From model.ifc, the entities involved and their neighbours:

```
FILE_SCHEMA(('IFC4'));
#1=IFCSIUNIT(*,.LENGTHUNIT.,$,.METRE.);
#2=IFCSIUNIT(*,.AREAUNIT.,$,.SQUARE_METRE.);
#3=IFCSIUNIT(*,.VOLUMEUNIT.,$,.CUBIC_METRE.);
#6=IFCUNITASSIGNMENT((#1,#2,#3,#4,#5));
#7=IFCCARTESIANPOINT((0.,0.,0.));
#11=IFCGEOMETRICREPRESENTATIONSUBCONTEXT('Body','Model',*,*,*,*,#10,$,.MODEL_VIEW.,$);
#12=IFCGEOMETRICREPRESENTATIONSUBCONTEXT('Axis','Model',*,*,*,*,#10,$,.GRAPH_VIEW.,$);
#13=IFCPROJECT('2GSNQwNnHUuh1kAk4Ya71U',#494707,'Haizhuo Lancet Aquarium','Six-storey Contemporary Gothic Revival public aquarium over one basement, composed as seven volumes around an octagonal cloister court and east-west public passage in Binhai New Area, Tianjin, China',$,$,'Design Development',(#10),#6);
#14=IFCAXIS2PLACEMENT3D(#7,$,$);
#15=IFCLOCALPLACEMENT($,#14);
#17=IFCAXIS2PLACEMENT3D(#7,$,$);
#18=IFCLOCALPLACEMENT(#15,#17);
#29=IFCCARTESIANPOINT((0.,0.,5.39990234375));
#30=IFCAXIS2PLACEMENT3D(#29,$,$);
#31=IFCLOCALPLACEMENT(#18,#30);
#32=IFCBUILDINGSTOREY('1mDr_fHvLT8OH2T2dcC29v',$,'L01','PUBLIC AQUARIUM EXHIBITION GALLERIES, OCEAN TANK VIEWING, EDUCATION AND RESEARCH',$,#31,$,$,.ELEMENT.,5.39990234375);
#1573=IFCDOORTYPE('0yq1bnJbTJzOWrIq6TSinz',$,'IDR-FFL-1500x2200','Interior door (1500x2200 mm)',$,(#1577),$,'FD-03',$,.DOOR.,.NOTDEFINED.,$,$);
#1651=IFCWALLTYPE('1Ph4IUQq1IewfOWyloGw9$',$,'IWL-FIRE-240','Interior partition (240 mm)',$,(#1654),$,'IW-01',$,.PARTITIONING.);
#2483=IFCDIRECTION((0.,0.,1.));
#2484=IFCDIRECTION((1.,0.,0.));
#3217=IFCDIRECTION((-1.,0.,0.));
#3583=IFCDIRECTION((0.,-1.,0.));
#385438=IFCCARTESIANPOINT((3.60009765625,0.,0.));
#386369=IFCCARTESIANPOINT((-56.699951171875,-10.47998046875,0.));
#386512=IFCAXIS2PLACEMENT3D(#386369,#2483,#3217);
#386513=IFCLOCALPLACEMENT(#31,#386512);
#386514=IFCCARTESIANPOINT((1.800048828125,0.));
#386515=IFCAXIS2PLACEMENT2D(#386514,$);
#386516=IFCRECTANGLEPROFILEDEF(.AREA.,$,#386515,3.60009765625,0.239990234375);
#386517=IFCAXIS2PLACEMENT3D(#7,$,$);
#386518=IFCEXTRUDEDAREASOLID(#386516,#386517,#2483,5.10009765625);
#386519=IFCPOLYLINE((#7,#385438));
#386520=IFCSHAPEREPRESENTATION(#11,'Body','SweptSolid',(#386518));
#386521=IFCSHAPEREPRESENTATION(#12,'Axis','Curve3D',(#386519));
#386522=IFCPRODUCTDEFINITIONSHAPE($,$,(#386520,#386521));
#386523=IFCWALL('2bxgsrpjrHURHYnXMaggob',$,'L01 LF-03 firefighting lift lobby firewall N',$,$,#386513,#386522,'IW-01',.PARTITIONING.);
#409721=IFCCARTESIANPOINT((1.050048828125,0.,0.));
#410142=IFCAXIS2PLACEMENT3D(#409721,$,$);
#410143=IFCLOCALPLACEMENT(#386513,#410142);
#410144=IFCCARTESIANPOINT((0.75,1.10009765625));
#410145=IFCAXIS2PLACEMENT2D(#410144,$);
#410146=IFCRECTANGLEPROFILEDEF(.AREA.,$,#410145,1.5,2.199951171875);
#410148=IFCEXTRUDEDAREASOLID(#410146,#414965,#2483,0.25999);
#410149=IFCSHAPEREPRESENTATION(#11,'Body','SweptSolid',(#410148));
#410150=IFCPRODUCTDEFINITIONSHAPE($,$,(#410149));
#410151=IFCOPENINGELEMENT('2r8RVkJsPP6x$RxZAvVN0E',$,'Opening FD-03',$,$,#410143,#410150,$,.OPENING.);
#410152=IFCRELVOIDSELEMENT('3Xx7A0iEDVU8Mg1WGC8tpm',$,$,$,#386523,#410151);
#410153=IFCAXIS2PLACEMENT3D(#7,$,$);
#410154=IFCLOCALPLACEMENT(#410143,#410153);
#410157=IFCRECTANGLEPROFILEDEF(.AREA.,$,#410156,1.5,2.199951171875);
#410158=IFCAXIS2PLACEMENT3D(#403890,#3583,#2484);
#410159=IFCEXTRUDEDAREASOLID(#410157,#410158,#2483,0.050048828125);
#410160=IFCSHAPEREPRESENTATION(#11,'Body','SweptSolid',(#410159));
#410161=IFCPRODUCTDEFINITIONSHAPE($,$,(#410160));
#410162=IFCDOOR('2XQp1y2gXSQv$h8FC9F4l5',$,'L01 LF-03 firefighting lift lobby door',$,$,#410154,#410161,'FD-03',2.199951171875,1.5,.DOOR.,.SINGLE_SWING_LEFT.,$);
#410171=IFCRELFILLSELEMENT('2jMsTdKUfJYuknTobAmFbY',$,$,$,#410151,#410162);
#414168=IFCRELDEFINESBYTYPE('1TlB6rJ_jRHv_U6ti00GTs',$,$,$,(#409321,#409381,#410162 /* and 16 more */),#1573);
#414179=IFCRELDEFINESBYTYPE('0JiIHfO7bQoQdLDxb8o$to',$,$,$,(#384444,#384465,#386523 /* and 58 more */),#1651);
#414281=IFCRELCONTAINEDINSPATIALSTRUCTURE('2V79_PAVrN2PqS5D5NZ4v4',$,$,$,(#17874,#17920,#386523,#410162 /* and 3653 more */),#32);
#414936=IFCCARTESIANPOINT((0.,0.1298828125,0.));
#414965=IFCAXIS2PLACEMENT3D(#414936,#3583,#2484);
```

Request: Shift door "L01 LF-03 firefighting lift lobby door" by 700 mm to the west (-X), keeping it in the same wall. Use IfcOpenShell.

```python
import ifcopenshell
import ifcopenshell.api.geometry
import ifcopenshell.util.placement
import ifcopenshell.util.unit

model = ifcopenshell.open("model.ifc")
unit_scale = ifcopenshell.util.unit.calculate_unit_scale(model)

door = model.by_id(410162)
opening = door.FillsVoids[0].RelatingOpeningElement
wall = opening.VoidsElements[0].RelatingBuildingElement

wall_matrix = ifcopenshell.util.placement.get_local_placement(wall.ObjectPlacement)
shift = wall_matrix[:3, 0] * 0.7 / unit_scale
before = ifcopenshell.util.placement.get_local_placement(door.ObjectPlacement)[:3, 3].copy()

# The door is placed relative to its opening, so it follows when the opening moves.
matrix = ifcopenshell.util.placement.get_local_placement(opening.ObjectPlacement)
matrix[:3, 3] += shift
ifcopenshell.api.geometry.edit_object_placement(
    model, product=opening, matrix=matrix, is_si=False, should_transform_children=True
)

after = ifcopenshell.util.placement.get_local_placement(door.ObjectPlacement)[:3, 3]
print("door moved by", (after - before).round(3) + 0.0)

model.write("model_updated.ifc")
```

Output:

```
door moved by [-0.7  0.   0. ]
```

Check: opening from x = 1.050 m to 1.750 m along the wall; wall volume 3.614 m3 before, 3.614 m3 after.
